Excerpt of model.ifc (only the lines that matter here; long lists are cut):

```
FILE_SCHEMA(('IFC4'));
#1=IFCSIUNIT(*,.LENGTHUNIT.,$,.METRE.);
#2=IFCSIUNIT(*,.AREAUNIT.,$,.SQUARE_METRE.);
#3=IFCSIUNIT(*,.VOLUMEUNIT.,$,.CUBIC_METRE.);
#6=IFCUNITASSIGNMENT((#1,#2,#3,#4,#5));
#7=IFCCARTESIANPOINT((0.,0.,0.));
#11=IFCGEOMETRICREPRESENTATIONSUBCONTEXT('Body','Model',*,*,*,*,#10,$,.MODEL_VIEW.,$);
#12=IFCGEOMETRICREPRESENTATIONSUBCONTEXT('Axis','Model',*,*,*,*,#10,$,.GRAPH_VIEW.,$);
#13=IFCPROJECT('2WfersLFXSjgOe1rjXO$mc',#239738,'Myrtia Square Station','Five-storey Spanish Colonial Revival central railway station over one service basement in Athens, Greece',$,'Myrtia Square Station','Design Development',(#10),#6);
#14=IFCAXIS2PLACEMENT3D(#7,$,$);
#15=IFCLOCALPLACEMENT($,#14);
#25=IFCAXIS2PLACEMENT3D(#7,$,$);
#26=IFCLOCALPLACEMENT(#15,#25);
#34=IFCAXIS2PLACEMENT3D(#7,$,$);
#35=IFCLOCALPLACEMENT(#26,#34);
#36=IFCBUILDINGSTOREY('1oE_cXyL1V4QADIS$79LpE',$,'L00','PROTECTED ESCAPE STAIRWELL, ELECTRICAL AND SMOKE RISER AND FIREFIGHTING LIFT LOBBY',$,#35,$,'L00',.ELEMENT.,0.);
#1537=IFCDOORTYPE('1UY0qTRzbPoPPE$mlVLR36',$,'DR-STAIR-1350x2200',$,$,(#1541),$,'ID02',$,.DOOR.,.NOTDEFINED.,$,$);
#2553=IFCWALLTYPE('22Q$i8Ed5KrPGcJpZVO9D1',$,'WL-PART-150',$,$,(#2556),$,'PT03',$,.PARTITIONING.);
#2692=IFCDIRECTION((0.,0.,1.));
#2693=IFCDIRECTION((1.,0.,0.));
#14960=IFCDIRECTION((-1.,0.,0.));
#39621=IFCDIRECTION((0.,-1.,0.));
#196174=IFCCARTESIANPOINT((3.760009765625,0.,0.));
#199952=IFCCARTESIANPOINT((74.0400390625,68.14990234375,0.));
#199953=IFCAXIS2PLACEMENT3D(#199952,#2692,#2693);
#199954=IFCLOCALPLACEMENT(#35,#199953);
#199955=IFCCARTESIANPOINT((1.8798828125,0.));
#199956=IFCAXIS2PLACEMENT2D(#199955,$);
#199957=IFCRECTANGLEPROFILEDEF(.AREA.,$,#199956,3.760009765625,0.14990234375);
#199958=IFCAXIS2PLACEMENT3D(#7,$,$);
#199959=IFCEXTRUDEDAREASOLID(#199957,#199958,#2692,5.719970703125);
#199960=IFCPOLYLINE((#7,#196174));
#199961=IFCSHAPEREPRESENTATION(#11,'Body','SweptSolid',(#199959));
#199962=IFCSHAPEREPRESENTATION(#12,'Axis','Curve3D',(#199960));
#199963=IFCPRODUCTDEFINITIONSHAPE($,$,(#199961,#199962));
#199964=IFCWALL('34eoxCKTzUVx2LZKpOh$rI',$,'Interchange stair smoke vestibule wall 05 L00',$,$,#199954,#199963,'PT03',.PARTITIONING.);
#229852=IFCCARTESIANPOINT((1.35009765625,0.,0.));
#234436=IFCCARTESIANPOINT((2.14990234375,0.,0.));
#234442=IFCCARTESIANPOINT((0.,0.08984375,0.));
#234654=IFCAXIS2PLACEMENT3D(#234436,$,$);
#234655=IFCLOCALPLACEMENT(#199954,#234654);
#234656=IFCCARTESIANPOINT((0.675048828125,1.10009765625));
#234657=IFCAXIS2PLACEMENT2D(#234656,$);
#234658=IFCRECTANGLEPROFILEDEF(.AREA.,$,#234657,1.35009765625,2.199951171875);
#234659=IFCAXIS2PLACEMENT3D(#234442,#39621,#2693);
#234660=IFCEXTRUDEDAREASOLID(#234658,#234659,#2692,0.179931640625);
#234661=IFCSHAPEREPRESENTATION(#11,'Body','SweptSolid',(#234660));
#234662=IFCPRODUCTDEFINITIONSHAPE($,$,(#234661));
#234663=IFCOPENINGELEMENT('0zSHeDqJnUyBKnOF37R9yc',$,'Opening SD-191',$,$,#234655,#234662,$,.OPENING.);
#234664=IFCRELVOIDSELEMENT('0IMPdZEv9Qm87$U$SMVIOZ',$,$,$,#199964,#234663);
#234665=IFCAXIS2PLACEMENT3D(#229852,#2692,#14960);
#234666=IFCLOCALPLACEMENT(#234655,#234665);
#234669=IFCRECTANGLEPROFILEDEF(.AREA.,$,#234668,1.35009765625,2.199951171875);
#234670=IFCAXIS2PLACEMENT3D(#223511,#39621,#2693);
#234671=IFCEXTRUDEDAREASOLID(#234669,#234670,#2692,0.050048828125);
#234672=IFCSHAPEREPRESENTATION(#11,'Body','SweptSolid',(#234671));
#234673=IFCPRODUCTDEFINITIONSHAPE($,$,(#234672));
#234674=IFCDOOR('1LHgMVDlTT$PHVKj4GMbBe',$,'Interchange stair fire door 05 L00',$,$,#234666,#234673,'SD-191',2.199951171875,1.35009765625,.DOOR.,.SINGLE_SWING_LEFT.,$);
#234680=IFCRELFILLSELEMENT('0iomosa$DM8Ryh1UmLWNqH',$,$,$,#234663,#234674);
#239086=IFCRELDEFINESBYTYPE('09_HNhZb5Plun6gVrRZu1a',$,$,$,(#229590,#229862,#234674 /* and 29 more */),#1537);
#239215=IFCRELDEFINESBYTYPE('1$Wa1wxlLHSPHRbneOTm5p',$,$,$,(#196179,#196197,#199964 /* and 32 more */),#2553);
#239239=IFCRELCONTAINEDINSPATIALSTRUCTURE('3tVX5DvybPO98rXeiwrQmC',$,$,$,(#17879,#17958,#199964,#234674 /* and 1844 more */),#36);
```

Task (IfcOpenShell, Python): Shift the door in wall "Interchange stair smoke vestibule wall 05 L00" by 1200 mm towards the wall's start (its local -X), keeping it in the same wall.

```python
import ifcopenshell
import ifcopenshell.api.geometry
import ifcopenshell.util.placement

model = ifcopenshell.open("model.ifc")

door = model.by_guid("1LHgMVDlTT$PHVKj4GMbBe")
opening = door.FillsVoids[0].RelatingOpeningElement
wall = opening.VoidsElements[0].RelatingBuildingElement

wall_matrix = ifcopenshell.util.placement.get_local_placement(wall.ObjectPlacement)
shift = wall_matrix[:3, 0] * -1.2
before = ifcopenshell.util.placement.get_local_placement(door.ObjectPlacement)[:3, 3].copy()

# The door is placed relative to its opening, so it follows when the opening moves.
matrix = ifcopenshell.util.placement.get_local_placement(opening.ObjectPlacement)
matrix[:3, 3] += shift
ifcopenshell.api.geometry.edit_object_placement(
    model, product=opening, matrix=matrix, is_si=False, should_transform_children=True
)

after = ifcopenshell.util.placement.get_local_placement(door.ObjectPlacement)[:3, 3]
print("door moved by", (after - before).round(3) + 0.0)

model.write("model_v2.ifc")
```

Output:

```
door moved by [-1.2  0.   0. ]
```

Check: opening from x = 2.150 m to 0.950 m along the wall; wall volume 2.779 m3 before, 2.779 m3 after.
